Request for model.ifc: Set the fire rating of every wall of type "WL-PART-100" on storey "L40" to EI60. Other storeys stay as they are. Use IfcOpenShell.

First a look at what the model holds.

```python
import ifcopenshell
import ifcopenshell.util.element

model = ifcopenshell.open("model.ifc")
print(model.schema)
storey = next(s for s in model.by_type("IfcBuildingStorey") if s.Name == "L40")
walls = [e for e in ifcopenshell.util.element.get_decomposition(storey) if e.is_a("IfcWall")]
seen = {}
for e in walls:
    element_type = ifcopenshell.util.element.get_type(e)
    key = (element_type.Name if element_type != e and element_type else None, ifcopenshell.util.element.get_pset(e, "Pset_WallCommon", "FireRating"))
    seen[key] = seen.get(key, 0) + 1
for (name, value), count in sorted(seen.items(), key=str):
    print(count, "x", name, "|", value)
```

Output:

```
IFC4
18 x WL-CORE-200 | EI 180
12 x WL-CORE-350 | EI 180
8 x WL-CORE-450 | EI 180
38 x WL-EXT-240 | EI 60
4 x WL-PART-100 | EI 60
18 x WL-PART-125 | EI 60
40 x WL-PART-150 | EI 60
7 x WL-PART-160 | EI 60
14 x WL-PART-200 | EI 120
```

```python
import ifcopenshell
import ifcopenshell.api.pset
import ifcopenshell.util.element

model = ifcopenshell.open("model.ifc")

storey = next(s for s in model.by_type("IfcBuildingStorey") if s.Name == "L40")
walls = [e for e in ifcopenshell.util.element.get_decomposition(storey) if e.is_a("IfcWall")]

count = 0
for e in walls:
    element_type = ifcopenshell.util.element.get_type(e)
    if element_type in (None, e) or element_type.Name != "WL-PART-100":
        continue
    found = ifcopenshell.util.element.get_pset(e, "Pset_WallCommon", should_inherit=False)
    if found:
        pset = model.by_id(found["id"])
        if len(ifcopenshell.util.element.get_elements_by_pset(pset)) > 1:
            pset = ifcopenshell.api.pset.unshare_pset(model, products=[e], pset=pset)[0]
    else:
        pset = ifcopenshell.api.pset.add_pset(model, product=e, name="Pset_WallCommon")
    ifcopenshell.api.pset.edit_pset(model, pset=pset, properties={"FireRating": "EI60"})
    count += 1

print(count, "walls updated")

model.write("model-out.ifc")
```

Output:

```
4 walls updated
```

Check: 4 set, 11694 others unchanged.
